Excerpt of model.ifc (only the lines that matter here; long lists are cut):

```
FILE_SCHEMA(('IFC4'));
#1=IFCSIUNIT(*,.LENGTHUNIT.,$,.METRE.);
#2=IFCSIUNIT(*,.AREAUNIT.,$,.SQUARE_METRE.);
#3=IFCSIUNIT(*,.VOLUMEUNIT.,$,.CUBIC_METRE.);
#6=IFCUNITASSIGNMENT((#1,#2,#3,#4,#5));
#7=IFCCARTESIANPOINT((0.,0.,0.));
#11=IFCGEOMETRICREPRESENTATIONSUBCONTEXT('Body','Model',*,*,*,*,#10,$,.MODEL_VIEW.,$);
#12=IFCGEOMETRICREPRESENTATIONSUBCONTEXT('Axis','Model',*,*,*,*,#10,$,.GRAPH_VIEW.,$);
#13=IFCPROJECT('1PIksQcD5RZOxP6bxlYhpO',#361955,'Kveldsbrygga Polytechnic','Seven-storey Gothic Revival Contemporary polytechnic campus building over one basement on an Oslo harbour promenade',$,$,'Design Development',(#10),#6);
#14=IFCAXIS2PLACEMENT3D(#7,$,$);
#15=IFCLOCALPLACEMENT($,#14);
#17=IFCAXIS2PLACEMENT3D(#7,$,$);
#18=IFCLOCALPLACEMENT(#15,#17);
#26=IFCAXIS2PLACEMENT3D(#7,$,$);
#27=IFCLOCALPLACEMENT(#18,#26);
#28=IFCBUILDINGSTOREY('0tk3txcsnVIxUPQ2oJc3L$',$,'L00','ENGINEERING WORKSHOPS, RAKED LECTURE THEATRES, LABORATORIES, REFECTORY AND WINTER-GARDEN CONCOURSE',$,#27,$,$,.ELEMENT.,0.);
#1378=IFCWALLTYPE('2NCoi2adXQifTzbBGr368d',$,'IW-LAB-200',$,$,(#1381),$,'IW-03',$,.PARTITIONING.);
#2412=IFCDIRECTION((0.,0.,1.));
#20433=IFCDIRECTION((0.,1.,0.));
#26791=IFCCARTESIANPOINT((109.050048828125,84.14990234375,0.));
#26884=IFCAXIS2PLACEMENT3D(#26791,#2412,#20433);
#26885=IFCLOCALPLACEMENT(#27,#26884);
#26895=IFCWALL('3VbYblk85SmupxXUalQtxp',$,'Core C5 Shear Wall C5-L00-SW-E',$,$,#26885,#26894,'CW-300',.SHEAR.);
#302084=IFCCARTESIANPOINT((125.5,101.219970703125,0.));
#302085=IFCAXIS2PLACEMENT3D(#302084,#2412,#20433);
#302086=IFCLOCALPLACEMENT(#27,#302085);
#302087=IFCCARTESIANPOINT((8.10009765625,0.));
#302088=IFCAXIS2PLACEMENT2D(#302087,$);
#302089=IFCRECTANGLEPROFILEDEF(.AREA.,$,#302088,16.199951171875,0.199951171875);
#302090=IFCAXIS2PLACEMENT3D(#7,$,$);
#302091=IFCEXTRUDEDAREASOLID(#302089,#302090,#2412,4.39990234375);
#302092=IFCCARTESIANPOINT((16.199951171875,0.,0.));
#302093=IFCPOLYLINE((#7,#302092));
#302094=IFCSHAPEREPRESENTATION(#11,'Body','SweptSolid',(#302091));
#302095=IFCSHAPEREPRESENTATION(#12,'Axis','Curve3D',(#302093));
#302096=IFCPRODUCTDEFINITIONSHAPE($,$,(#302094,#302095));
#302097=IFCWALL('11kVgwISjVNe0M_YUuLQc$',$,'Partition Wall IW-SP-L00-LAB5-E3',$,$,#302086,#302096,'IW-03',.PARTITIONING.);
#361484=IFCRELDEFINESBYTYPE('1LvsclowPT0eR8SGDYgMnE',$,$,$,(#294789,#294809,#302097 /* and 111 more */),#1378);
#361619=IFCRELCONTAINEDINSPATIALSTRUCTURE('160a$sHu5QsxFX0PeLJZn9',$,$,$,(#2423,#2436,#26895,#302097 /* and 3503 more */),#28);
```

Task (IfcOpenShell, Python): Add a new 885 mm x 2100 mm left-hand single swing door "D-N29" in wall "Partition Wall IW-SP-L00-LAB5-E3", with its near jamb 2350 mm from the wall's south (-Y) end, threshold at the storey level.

```python
import numpy as np
import ifcopenshell
import ifcopenshell.api.feature
import ifcopenshell.api.geometry
import ifcopenshell.api.root
import ifcopenshell.api.spatial
import ifcopenshell.geom
import ifcopenshell.util.element
import ifcopenshell.util.placement
import ifcopenshell.util.representation
import ifcopenshell.util.shape
import ifcopenshell.util.unit

model = ifcopenshell.open("model.ifc")
unit_scale = ifcopenshell.util.unit.calculate_unit_scale(model)
settings = ifcopenshell.geom.settings()


def volume(element):
    """Net volume in cubic metres, openings subtracted."""
    shape = ifcopenshell.geom.create_shape(settings, element)
    return ifcopenshell.util.shape.get_volume(shape.geometry)


wall = model.by_guid("11kVgwISjVNe0M_YUuLQc$")
storey = ifcopenshell.util.element.get_container(wall, ifc_class="IfcBuildingStorey")
context = ifcopenshell.util.representation.get_context(model, "Model", "Body", "MODEL_VIEW")
before = volume(wall)

width, height, from_end, sill = 0.885, 2.1, 2.35, 0.0  # metres

# The wall runs along its own X axis, and the end named is its -X end.
wall_shape = ifcopenshell.geom.create_shape(settings, wall)
x, y, z = ifcopenshell.util.shape.get_vertices(wall_shape.geometry).T
start = x.min() + from_end
face, thickness = float(y.min()), float(y.max() - y.min())
wall_matrix = ifcopenshell.util.placement.get_local_placement(wall.ObjectPlacement)
level = ifcopenshell.util.placement.get_local_placement(storey.ObjectPlacement)[2, 3]


def in_wall(x, y):
    """Placement at x, y metres in the wall's axes, at sill height."""
    matrix = wall_matrix.copy()
    matrix[:, 3] = wall_matrix @ np.array([x / unit_scale, y / unit_scale, 0.0, 1.0])
    matrix[2, 3] = level + sill / unit_scale
    return matrix


# Opening: a box that overshoots both wall faces by 50 mm.
opening = ifcopenshell.api.root.create_entity(model, ifc_class="IfcOpeningElement", predefined_type="OPENING")
box = ifcopenshell.api.geometry.add_wall_representation(
    model, context=context, length=width, height=height, thickness=thickness + 0.1
)
ifcopenshell.api.geometry.assign_representation(model, product=opening, representation=box)
ifcopenshell.api.geometry.edit_object_placement(model, product=opening, matrix=in_wall(start, face - 0.05), is_si=False)
ifcopenshell.api.feature.add_feature(model, feature=opening, element=wall)

door = ifcopenshell.api.root.create_entity(model, ifc_class="IfcDoor", name="D-N29", predefined_type="DOOR")
door.OverallWidth, door.OverallHeight = width / unit_scale, height / unit_scale
door.OperationType = "SINGLE_SWING_LEFT"
body = ifcopenshell.api.geometry.add_door_representation(
    model,
    context=context,
    overall_width=door.OverallWidth,
    overall_height=door.OverallHeight,
    operation_type="SINGLE_SWING_LEFT",
    lining_properties={"LiningDepth": thickness / unit_scale, "ThresholdDepth": thickness / unit_scale},
)
ifcopenshell.api.geometry.assign_representation(model, product=door, representation=body)
ifcopenshell.api.spatial.assign_container(model, products=[door], relating_structure=storey)
ifcopenshell.api.feature.add_filling(model, opening=opening, element=door)

# The lining spans the wall, so the door starts at the wall face.
ifcopenshell.api.geometry.edit_object_placement(model, product=door, matrix=in_wall(start, face), is_si=False)

after = volume(wall)

print(f"wall volume {before:.3f} -> {after:.3f} m3")

model.write("model_rev.ifc")
```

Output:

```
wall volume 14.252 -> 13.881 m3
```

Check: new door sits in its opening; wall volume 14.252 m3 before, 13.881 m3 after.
